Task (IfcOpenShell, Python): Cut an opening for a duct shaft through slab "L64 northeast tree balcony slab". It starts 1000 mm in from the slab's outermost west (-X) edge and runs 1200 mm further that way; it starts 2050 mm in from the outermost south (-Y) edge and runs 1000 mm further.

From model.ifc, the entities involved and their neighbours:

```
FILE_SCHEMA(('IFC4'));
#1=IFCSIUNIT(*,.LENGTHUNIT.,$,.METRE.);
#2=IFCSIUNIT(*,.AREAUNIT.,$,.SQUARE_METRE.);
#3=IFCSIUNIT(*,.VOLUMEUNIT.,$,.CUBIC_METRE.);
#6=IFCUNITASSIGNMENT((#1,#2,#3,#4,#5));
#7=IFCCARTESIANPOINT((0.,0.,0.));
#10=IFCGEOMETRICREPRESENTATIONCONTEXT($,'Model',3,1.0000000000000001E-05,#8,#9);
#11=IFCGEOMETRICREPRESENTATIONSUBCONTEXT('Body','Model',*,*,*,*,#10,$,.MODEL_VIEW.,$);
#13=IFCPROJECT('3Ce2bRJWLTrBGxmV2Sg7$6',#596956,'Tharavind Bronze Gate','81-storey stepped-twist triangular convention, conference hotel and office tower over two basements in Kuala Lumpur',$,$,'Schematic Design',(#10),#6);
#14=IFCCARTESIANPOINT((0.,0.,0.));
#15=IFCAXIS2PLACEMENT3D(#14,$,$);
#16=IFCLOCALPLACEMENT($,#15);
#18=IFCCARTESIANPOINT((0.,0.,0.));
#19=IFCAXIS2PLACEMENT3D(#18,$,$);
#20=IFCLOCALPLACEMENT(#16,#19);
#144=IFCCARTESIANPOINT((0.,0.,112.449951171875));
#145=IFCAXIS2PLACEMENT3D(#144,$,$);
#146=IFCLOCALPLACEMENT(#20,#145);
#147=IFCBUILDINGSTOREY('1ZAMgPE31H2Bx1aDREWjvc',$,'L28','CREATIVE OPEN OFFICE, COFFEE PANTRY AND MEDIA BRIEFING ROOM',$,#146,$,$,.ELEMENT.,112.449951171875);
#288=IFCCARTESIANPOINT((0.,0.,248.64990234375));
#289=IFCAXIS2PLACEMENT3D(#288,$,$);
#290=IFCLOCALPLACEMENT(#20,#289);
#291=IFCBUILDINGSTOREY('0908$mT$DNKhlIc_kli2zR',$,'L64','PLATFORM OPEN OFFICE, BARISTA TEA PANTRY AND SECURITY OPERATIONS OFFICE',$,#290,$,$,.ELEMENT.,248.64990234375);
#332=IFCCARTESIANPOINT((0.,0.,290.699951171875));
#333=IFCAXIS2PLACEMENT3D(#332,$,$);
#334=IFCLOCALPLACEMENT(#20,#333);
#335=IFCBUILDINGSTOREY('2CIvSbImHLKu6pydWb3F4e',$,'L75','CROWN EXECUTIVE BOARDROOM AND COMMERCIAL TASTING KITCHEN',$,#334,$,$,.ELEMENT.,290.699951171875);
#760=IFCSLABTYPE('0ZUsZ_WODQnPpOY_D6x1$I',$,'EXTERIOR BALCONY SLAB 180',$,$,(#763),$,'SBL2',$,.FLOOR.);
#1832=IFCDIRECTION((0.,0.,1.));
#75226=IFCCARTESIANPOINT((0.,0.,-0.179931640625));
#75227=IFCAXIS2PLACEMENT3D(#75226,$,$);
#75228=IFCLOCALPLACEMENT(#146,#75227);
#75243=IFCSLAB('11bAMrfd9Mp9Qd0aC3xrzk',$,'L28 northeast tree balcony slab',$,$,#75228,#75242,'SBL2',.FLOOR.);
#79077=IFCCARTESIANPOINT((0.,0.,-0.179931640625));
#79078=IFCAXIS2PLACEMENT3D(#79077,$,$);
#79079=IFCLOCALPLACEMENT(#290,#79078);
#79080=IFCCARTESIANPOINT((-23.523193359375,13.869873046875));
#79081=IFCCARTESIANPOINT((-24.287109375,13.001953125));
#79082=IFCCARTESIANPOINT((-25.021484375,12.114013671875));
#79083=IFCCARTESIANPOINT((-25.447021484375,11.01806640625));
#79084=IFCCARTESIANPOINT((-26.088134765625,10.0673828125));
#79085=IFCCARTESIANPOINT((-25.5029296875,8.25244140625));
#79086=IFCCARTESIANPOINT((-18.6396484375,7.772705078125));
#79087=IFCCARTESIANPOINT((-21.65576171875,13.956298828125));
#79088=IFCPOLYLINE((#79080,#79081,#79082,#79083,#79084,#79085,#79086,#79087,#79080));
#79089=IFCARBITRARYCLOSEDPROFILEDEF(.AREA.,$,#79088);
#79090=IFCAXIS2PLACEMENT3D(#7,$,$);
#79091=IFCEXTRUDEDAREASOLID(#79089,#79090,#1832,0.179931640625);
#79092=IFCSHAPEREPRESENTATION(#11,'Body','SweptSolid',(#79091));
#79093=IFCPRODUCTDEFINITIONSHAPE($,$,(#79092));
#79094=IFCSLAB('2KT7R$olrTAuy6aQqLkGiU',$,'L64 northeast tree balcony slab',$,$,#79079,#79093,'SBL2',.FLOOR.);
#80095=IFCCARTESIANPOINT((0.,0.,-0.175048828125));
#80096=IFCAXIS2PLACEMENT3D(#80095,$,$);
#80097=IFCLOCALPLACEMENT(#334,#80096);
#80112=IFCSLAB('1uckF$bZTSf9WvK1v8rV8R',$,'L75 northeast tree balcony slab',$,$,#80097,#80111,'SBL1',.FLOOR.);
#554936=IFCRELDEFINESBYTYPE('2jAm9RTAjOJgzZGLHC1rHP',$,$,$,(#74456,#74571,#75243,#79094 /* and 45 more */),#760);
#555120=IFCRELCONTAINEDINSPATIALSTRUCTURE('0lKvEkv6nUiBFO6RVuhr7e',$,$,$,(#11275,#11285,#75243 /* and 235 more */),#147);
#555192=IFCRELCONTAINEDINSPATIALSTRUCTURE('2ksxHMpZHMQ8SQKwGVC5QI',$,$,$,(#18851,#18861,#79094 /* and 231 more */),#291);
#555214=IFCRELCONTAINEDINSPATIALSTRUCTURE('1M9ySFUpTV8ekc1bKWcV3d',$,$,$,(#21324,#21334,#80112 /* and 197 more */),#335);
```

```python
import numpy as np
import ifcopenshell
import ifcopenshell.api.feature
import ifcopenshell.api.geometry
import ifcopenshell.api.root
import ifcopenshell.geom
import ifcopenshell.util.placement
import ifcopenshell.util.representation
import ifcopenshell.util.shape
import ifcopenshell.util.unit

model = ifcopenshell.open("model.ifc")
unit_scale = ifcopenshell.util.unit.calculate_unit_scale(model)
settings = ifcopenshell.geom.settings()


def volume(element):
    """Net volume in cubic metres, openings subtracted."""
    shape = ifcopenshell.geom.create_shape(settings, element)
    return ifcopenshell.util.shape.get_volume(shape.geometry)


slab = model.by_id(79094)
before = volume(slab)

# Extent in the slab's own axes, in metres. The edges named are its -X and -Y sides.
slab_shape = ifcopenshell.geom.create_shape(settings, slab)
vertices = ifcopenshell.util.shape.get_vertices(slab_shape.geometry)
x_min, y_min, bottom = vertices.min(axis=0)
top = vertices[:, 2].max()

opening = ifcopenshell.api.root.create_entity(model, ifc_class="IfcOpeningElement", name="Duct shaft opening", predefined_type="OPENING")
context = ifcopenshell.util.representation.get_context(model, "Model", "Body", "MODEL_VIEW")
width, depth = 1.2, 1
outline = [(0.0, 0.0), (width, 0.0), (width, depth), (0.0, depth), (0.0, 0.0)]
# Overshoot both faces by 50 mm so the cut is clean.
shape = ifcopenshell.api.geometry.add_slab_representation(
    model, context=context, depth=top - bottom + 0.1, polyline=outline
)
ifcopenshell.api.geometry.assign_representation(model, product=opening, representation=shape)

matrix = ifcopenshell.util.placement.get_local_placement(slab.ObjectPlacement)
matrix[:, 3] = matrix @ np.append(np.array([x_min + 1, y_min + 2.05, bottom - 0.05]) / unit_scale, 1.0)
ifcopenshell.api.geometry.edit_object_placement(model, product=opening, matrix=matrix, is_si=False)
ifcopenshell.api.feature.add_feature(model, feature=opening, element=slab)

after = volume(slab)

print(f"slab volume {before:.3f} -> {after:.3f} m3")

model.write("model-out.ifc")
```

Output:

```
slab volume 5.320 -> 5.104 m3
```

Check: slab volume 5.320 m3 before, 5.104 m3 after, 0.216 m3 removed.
